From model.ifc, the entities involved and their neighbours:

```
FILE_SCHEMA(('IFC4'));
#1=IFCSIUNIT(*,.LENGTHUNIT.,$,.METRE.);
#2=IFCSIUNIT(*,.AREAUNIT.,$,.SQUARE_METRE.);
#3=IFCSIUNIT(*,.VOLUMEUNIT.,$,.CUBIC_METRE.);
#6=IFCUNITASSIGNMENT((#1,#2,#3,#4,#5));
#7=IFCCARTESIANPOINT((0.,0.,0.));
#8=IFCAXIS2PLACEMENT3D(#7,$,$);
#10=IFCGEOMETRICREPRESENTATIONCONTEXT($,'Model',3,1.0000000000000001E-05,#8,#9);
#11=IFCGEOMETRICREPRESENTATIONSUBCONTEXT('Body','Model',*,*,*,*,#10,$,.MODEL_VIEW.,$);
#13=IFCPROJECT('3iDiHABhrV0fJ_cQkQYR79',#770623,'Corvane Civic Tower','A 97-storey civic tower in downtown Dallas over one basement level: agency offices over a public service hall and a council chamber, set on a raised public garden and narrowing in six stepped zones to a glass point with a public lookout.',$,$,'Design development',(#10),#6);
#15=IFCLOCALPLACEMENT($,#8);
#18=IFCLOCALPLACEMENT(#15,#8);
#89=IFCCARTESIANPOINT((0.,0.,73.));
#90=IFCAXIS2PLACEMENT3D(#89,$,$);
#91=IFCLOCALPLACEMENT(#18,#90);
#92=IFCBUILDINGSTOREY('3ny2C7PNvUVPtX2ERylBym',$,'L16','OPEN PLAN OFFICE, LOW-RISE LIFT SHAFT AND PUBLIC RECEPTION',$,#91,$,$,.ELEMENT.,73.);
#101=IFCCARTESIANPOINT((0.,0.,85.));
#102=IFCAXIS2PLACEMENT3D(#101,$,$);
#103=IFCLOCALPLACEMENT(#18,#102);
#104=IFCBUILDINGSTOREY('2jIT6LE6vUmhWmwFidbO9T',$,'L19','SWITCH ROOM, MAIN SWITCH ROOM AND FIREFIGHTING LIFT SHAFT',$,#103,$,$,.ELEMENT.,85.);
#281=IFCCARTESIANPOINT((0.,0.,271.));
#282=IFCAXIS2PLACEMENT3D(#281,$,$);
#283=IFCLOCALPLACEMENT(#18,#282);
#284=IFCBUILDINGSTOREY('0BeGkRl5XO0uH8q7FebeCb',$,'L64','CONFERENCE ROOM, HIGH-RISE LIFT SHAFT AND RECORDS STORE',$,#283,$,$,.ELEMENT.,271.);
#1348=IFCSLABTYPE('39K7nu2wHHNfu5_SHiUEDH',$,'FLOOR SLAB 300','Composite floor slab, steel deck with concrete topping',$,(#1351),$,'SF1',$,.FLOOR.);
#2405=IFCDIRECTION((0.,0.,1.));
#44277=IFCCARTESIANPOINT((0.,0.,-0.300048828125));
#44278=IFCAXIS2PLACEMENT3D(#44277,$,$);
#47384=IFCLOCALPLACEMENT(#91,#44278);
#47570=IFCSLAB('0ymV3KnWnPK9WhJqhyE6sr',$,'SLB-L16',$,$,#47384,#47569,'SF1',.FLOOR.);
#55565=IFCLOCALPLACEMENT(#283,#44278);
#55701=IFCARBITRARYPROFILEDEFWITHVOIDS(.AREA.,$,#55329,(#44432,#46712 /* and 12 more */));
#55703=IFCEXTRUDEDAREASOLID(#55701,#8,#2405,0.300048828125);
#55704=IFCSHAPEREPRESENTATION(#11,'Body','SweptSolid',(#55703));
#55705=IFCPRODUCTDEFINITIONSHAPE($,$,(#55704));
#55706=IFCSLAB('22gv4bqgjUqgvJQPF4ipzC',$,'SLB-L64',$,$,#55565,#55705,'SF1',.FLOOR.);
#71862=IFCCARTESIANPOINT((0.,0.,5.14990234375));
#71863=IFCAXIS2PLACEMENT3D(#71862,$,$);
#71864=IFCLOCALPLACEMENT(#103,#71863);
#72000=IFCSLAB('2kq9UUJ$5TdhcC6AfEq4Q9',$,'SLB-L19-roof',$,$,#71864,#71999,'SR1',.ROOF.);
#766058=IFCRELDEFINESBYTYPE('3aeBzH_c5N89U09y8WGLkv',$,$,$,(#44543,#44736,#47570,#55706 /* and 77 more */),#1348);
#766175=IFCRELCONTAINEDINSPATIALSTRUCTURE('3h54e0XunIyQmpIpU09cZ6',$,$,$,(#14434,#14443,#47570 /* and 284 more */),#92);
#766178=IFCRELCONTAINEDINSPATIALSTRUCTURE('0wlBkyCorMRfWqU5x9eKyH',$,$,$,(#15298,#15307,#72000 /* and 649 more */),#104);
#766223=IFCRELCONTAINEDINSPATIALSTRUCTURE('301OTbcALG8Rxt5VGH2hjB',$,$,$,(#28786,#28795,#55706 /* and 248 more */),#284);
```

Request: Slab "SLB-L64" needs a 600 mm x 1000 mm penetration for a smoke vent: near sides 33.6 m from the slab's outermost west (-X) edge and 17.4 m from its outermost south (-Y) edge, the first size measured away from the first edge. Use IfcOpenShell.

```python
import numpy as np
import ifcopenshell
import ifcopenshell.api.feature
import ifcopenshell.api.geometry
import ifcopenshell.api.root
import ifcopenshell.geom
import ifcopenshell.util.placement
import ifcopenshell.util.representation
import ifcopenshell.util.shape
import ifcopenshell.util.unit

model = ifcopenshell.open("model.ifc")
unit_scale = ifcopenshell.util.unit.calculate_unit_scale(model)
settings = ifcopenshell.geom.settings()


def volume(element):
    """Net volume in cubic metres, openings subtracted."""
    shape = ifcopenshell.geom.create_shape(settings, element)
    return ifcopenshell.util.shape.get_volume(shape.geometry)


slab = model.by_id(55706)
before = volume(slab)

# Extent in the slab's own axes, in metres. The edges named are its -X and -Y sides.
slab_shape = ifcopenshell.geom.create_shape(settings, slab)
vertices = ifcopenshell.util.shape.get_vertices(slab_shape.geometry)
x_min, y_min, bottom = vertices.min(axis=0)
top = vertices[:, 2].max()

opening = ifcopenshell.api.root.create_entity(model, ifc_class="IfcOpeningElement", name="Smoke vent opening", predefined_type="OPENING")
context = ifcopenshell.util.representation.get_context(model, "Model", "Body", "MODEL_VIEW")
width, depth = 0.6, 1
outline = [(0.0, 0.0), (width, 0.0), (width, depth), (0.0, depth), (0.0, 0.0)]
# Overshoot both faces by 50 mm so the cut is clean.
shape = ifcopenshell.api.geometry.add_slab_representation(
    model, context=context, depth=top - bottom + 0.1, polyline=outline
)
ifcopenshell.api.geometry.assign_representation(model, product=opening, representation=shape)

matrix = ifcopenshell.util.placement.get_local_placement(slab.ObjectPlacement)
matrix[:, 3] = matrix @ np.append(np.array([x_min + 33.6, y_min + 17.4, bottom - 0.05]) / unit_scale, 1.0)
ifcopenshell.api.geometry.edit_object_placement(model, product=opening, matrix=matrix, is_si=False)
ifcopenshell.api.feature.add_feature(model, feature=opening, element=slab)

after = volume(slab)

print(f"slab volume {before:.3f} -> {after:.3f} m3")

model.write("model-out.ifc")
```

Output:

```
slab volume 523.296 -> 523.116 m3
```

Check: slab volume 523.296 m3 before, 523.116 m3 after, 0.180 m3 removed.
